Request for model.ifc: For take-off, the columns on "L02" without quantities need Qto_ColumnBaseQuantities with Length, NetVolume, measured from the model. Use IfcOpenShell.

First a look at what the model holds.

```python
import ifcopenshell
import ifcopenshell.util.element
import ifcopenshell.util.unit

model = ifcopenshell.open("model.ifc")
print(model.schema)
for unit_type in ("LENGTHUNIT", "AREAUNIT", "VOLUMEUNIT"):
    print(unit_type, ifcopenshell.util.unit.calculate_unit_scale(model, unit_type))
storey = next(s for s in model.by_type("IfcBuildingStorey") if s.Name == "L02")
columns = [e for e in ifcopenshell.util.element.get_decomposition(storey) if e.is_a("IfcColumn")]
for e in sorted(columns, key=lambda e: e.id()):
    print(e.id(), e.is_a(), e.Name, list(ifcopenshell.util.element.get_psets(e, qtos_only=True)), sep=" | ")
```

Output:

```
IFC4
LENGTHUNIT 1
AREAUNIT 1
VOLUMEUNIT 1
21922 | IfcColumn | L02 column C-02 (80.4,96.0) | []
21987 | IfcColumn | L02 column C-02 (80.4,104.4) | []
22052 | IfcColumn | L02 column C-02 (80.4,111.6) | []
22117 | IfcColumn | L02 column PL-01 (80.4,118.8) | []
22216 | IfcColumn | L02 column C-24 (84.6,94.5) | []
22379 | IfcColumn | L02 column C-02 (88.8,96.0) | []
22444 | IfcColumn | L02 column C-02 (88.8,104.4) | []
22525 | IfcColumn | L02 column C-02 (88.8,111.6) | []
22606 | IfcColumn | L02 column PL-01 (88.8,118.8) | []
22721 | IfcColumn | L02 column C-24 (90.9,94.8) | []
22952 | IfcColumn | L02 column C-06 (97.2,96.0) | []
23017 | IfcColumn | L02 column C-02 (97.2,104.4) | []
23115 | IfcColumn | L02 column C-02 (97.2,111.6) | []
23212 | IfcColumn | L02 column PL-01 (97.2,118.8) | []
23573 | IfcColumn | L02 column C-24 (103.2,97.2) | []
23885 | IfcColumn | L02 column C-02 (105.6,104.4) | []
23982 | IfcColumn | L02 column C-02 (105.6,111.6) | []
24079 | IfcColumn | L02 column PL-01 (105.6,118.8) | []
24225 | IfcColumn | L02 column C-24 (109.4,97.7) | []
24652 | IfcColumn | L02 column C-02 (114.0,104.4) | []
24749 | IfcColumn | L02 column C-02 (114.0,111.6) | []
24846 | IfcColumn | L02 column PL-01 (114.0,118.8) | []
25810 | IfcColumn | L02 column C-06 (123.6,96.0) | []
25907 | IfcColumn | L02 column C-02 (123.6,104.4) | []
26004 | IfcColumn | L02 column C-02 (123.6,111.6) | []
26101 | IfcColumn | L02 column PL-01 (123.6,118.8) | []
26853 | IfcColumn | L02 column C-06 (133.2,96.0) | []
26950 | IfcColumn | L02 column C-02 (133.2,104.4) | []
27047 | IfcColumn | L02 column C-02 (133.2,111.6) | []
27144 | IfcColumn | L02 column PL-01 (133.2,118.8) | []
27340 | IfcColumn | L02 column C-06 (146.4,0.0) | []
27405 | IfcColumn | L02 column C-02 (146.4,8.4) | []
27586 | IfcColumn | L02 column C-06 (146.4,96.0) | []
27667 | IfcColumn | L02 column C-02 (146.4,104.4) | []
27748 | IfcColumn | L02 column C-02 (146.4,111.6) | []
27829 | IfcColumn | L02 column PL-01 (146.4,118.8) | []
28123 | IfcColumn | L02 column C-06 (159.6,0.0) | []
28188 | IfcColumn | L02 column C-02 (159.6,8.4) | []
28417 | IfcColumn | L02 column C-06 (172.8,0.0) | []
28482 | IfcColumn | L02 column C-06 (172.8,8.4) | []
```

```python
import ifcopenshell
import ifcopenshell.api.pset
import ifcopenshell.geom
import ifcopenshell.util.element
import ifcopenshell.util.shape
import ifcopenshell.util.unit

model = ifcopenshell.open("model.ifc")
unit_scale = ifcopenshell.util.unit.calculate_unit_scale(model)
volume_scale = ifcopenshell.util.unit.calculate_unit_scale(model, "VOLUMEUNIT")
settings = ifcopenshell.geom.settings()

storey = next(s for s in model.by_type("IfcBuildingStorey") if s.Name == "L02")
columns = [e for e in ifcopenshell.util.element.get_decomposition(storey) if e.is_a("IfcColumn")]

for e in sorted(columns, key=lambda e: e.id()):
    if ifcopenshell.util.element.get_psets(e, qtos_only=True, should_inherit=False):
        continue
    # Geometry comes back in metres, in the element's own axes.
    shape = ifcopenshell.geom.create_shape(settings, e)
    values = {
        "Length": ifcopenshell.util.shape.get_z(shape.geometry) / unit_scale,
        "NetVolume": ifcopenshell.util.shape.get_volume(shape.geometry) / volume_scale,
    }
    qto = ifcopenshell.api.pset.add_qto(model, product=e, name="Qto_ColumnBaseQuantities")
    ifcopenshell.api.pset.edit_qto(model, qto=qto, properties=values)
    print(e.id(), {k: round(v, 3) for k, v in values.items()})

model.write("model_edited.ifc")
```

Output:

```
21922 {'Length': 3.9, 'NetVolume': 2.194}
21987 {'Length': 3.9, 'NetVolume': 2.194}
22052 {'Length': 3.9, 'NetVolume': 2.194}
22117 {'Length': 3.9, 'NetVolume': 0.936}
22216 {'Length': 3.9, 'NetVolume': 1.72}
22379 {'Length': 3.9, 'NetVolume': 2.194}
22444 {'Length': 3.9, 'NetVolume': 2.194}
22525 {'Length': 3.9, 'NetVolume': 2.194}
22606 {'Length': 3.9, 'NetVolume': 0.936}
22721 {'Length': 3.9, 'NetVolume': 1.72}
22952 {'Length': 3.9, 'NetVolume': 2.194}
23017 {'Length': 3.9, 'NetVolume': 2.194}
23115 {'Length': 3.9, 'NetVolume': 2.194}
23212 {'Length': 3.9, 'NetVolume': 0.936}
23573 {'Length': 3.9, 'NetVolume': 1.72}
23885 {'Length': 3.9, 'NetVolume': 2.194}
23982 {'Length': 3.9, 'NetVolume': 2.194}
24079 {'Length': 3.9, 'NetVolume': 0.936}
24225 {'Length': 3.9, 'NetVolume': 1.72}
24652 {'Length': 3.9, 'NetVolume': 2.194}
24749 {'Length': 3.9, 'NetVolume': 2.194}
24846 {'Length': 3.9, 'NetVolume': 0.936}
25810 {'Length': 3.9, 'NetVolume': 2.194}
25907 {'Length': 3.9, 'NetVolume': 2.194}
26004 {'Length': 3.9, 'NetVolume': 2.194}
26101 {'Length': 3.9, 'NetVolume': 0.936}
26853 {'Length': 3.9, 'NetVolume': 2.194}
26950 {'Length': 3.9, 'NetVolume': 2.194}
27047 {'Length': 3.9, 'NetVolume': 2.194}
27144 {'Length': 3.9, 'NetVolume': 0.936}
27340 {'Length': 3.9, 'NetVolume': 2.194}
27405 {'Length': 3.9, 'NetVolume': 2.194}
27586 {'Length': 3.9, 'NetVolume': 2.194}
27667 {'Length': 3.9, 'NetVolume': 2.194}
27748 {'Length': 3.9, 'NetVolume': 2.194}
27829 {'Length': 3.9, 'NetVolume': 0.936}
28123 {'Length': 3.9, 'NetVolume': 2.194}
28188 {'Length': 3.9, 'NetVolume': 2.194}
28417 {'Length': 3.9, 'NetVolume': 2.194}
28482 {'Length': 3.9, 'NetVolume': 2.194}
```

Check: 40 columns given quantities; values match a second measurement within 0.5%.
